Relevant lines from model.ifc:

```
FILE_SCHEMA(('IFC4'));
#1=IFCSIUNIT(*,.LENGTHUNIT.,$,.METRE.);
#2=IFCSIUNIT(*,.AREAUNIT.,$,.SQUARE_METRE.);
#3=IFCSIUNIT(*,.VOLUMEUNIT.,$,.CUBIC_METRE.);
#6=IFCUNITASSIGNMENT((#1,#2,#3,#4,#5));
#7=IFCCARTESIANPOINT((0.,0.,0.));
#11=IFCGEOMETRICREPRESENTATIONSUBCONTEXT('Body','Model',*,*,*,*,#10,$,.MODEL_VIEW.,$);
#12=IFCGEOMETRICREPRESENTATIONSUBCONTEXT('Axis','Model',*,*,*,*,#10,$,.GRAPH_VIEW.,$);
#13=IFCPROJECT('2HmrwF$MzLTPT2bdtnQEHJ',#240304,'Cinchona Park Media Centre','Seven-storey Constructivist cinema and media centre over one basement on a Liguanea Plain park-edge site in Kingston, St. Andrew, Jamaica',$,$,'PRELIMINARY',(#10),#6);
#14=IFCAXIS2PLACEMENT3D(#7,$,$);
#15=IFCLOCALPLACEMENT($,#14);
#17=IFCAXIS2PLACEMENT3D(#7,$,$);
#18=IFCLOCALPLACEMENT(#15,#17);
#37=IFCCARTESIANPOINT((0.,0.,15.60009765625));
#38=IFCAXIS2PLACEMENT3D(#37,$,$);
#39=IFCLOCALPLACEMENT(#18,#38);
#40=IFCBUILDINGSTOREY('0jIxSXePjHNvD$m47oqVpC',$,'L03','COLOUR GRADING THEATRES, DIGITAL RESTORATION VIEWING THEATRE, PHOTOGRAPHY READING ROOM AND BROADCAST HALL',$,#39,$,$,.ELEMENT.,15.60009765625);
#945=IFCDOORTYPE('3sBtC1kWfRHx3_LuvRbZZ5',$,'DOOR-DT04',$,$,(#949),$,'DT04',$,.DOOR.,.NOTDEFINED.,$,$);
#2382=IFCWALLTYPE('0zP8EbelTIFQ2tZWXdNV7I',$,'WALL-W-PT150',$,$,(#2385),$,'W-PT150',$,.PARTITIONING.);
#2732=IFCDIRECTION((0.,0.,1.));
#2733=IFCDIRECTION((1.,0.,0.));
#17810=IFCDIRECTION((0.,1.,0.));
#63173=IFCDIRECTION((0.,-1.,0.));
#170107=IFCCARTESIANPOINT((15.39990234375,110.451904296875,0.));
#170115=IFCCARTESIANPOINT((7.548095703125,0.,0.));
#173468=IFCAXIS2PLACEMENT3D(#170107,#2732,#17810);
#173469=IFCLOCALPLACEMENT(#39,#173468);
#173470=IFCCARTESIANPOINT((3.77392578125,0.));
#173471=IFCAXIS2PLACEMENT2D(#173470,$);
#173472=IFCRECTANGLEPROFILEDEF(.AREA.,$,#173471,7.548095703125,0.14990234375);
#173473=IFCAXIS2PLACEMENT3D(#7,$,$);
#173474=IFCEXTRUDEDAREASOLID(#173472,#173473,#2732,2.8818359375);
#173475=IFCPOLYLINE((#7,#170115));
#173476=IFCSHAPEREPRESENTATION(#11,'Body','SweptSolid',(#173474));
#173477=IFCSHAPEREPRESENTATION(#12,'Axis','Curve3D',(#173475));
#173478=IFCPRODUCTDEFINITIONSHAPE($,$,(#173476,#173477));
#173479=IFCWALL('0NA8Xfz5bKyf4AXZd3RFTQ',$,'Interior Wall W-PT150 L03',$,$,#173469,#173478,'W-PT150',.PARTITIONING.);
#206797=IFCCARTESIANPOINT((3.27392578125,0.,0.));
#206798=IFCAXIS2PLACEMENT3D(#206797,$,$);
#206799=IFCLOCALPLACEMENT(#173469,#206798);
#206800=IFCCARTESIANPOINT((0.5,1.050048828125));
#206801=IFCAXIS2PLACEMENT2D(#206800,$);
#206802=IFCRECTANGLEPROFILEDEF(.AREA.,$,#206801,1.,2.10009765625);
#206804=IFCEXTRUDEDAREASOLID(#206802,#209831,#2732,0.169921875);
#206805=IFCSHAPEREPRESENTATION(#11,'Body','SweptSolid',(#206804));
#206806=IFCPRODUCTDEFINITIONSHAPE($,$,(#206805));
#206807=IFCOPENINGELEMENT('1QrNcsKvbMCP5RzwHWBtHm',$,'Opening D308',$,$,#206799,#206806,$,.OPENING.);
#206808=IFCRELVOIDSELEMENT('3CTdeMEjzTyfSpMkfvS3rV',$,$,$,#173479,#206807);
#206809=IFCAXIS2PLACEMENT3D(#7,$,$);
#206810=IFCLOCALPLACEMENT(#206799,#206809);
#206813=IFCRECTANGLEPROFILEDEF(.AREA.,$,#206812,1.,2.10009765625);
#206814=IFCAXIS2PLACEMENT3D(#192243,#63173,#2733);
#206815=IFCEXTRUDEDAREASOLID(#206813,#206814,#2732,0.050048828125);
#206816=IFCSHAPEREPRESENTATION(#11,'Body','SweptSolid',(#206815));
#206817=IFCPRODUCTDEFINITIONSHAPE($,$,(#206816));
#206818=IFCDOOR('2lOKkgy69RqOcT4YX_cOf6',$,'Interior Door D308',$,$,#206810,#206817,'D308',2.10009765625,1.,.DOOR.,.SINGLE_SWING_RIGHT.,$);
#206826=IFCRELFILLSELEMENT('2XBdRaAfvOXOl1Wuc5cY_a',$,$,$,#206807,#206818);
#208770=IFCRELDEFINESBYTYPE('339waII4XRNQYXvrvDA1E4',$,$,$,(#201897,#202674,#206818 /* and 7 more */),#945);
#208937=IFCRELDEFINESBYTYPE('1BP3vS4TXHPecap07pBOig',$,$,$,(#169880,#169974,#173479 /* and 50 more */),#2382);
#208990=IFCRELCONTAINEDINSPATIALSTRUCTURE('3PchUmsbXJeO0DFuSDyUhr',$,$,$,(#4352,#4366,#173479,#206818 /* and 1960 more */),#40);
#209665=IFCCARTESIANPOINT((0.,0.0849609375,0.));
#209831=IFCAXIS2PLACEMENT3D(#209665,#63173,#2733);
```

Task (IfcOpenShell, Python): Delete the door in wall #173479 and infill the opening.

```python
import ifcopenshell
import ifcopenshell.api.feature
import ifcopenshell.api.root
import ifcopenshell.geom
import ifcopenshell.util.shape

model = ifcopenshell.open("model.ifc")
settings = ifcopenshell.geom.settings()


def volume(element):
    """Net volume in cubic metres, openings subtracted."""
    shape = ifcopenshell.geom.create_shape(settings, element)
    return ifcopenshell.util.shape.get_volume(shape.geometry)


door = model.by_guid("2lOKkgy69RqOcT4YX_cOf6")
opening = door.FillsVoids[0].RelatingOpeningElement
wall = opening.VoidsElements[0].RelatingBuildingElement
before = volume(wall)

ifcopenshell.api.root.remove_product(model, product=door)
ifcopenshell.api.feature.remove_feature(model, feature=opening)

after = volume(wall)

print(f"wall volume {before:.3f} -> {after:.3f} m3")

model.write("model_rev.ifc")
```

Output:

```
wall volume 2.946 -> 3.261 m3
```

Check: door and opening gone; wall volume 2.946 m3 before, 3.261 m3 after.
